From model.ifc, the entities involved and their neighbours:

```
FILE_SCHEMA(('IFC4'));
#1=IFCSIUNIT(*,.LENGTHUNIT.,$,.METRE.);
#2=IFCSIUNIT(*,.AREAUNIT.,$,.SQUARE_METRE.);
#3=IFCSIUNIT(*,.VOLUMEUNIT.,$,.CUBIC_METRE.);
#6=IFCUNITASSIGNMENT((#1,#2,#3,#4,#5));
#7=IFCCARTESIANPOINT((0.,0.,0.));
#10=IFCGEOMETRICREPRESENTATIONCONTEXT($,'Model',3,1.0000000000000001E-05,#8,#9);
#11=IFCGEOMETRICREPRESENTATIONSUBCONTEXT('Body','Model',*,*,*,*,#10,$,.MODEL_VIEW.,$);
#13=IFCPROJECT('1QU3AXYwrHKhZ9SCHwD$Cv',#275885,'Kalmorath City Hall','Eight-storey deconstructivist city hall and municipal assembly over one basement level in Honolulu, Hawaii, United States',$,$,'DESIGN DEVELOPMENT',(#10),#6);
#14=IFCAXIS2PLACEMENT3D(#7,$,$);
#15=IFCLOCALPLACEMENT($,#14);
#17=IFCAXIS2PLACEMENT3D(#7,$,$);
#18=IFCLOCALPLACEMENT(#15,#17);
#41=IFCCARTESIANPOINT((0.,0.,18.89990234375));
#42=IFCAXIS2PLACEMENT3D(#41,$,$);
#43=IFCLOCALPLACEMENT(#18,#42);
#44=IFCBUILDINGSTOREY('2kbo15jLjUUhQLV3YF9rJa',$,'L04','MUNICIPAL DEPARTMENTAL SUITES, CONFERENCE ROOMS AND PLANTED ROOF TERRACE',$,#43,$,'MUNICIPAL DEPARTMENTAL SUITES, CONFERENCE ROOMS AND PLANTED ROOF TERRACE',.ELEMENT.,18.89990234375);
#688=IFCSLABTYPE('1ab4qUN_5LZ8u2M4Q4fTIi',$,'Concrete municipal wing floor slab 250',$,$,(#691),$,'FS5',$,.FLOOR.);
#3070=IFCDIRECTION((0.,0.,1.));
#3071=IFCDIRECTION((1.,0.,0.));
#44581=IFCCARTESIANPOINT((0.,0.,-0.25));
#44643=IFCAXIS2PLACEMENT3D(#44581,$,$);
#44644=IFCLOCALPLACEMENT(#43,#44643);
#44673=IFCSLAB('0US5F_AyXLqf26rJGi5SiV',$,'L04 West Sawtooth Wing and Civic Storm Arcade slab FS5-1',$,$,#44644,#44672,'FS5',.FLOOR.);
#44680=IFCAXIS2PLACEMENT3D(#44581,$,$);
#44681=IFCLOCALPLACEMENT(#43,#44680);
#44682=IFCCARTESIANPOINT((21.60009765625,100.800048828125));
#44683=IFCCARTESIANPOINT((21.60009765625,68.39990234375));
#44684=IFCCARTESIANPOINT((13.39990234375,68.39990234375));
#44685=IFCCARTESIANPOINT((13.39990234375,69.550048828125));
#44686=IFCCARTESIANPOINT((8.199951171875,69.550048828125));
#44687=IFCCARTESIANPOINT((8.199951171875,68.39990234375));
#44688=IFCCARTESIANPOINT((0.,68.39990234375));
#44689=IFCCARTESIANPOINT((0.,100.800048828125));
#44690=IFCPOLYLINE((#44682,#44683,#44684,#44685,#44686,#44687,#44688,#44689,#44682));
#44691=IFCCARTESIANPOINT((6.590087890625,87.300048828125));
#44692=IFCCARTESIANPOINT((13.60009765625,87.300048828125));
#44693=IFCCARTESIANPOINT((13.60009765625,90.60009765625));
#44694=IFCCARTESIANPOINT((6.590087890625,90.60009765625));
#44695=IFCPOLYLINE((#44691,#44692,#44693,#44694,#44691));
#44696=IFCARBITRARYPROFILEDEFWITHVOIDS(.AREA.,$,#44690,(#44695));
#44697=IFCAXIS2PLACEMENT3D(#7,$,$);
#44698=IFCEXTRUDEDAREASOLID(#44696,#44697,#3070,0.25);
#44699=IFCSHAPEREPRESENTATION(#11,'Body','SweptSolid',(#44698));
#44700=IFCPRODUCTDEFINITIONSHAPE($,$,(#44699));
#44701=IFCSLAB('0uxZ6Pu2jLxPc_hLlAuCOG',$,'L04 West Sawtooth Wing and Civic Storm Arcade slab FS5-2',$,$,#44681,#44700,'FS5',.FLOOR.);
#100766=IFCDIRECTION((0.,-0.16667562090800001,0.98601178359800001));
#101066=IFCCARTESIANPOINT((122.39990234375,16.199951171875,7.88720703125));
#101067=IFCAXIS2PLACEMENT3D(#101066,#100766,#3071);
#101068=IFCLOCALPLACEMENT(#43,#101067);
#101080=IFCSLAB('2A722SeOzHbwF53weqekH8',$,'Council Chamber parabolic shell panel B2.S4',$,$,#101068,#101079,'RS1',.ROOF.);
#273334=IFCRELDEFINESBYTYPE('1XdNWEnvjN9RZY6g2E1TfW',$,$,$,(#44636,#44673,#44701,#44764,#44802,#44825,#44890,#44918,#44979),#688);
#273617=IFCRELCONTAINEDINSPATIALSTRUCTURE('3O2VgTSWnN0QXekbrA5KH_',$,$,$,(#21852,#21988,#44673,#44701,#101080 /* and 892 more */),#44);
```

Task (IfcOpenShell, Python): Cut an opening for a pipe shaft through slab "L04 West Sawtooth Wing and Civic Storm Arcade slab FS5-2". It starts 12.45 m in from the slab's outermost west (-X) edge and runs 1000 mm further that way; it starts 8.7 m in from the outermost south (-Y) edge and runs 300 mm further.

```python
import numpy as np
import ifcopenshell
import ifcopenshell.api.feature
import ifcopenshell.api.geometry
import ifcopenshell.api.root
import ifcopenshell.geom
import ifcopenshell.util.placement
import ifcopenshell.util.representation
import ifcopenshell.util.shape
import ifcopenshell.util.unit

model = ifcopenshell.open("model.ifc")
unit_scale = ifcopenshell.util.unit.calculate_unit_scale(model)
settings = ifcopenshell.geom.settings()


def volume(element):
    """Net volume in cubic metres, openings subtracted."""
    shape = ifcopenshell.geom.create_shape(settings, element)
    return ifcopenshell.util.shape.get_volume(shape.geometry)


slab = model.by_guid("0uxZ6Pu2jLxPc_hLlAuCOG")
before = volume(slab)

# Extent in the slab's own axes, in metres. The edges named are its -X and -Y sides.
slab_shape = ifcopenshell.geom.create_shape(settings, slab)
vertices = ifcopenshell.util.shape.get_vertices(slab_shape.geometry)
x_min, y_min, bottom = vertices.min(axis=0)
top = vertices[:, 2].max()

opening = ifcopenshell.api.root.create_entity(model, ifc_class="IfcOpeningElement", name="Pipe shaft opening", predefined_type="OPENING")
context = ifcopenshell.util.representation.get_context(model, "Model", "Body", "MODEL_VIEW")
width, depth = 1, 0.3
outline = [(0.0, 0.0), (width, 0.0), (width, depth), (0.0, depth), (0.0, 0.0)]
# Overshoot both faces by 50 mm so the cut is clean.
shape = ifcopenshell.api.geometry.add_slab_representation(
    model, context=context, depth=top - bottom + 0.1, polyline=outline
)
ifcopenshell.api.geometry.assign_representation(model, product=opening, representation=shape)

matrix = ifcopenshell.util.placement.get_local_placement(slab.ObjectPlacement)
matrix[:, 3] = matrix @ np.append(np.array([x_min + 12.45, y_min + 8.7, bottom - 0.05]) / unit_scale, 1.0)
ifcopenshell.api.geometry.edit_object_placement(model, product=opening, matrix=matrix, is_si=False)
ifcopenshell.api.feature.add_feature(model, feature=opening, element=slab)

after = volume(slab)

print(f"slab volume {before:.3f} -> {after:.3f} m3")

model.write("model_updated.ifc")
```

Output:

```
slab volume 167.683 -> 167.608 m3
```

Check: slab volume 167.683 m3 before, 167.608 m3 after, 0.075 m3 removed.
